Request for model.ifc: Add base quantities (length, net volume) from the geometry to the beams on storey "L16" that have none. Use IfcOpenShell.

First a look at what the model holds.

```python
import ifcopenshell
import ifcopenshell.util.element
import ifcopenshell.util.unit

model = ifcopenshell.open("model.ifc")
print(model.schema)
for unit_type in ("LENGTHUNIT", "AREAUNIT", "VOLUMEUNIT"):
    print(unit_type, ifcopenshell.util.unit.calculate_unit_scale(model, unit_type))
storey = next(s for s in model.by_type("IfcBuildingStorey") if s.Name == "L16")
beams = [e for e in ifcopenshell.util.element.get_decomposition(storey) if e.is_a("IfcBeam")]
for e in sorted(beams, key=lambda e: e.id()):
    print(e.id(), e.is_a(), e.Name, list(ifcopenshell.util.element.get_psets(e, qtos_only=True)), sep=" | ")
```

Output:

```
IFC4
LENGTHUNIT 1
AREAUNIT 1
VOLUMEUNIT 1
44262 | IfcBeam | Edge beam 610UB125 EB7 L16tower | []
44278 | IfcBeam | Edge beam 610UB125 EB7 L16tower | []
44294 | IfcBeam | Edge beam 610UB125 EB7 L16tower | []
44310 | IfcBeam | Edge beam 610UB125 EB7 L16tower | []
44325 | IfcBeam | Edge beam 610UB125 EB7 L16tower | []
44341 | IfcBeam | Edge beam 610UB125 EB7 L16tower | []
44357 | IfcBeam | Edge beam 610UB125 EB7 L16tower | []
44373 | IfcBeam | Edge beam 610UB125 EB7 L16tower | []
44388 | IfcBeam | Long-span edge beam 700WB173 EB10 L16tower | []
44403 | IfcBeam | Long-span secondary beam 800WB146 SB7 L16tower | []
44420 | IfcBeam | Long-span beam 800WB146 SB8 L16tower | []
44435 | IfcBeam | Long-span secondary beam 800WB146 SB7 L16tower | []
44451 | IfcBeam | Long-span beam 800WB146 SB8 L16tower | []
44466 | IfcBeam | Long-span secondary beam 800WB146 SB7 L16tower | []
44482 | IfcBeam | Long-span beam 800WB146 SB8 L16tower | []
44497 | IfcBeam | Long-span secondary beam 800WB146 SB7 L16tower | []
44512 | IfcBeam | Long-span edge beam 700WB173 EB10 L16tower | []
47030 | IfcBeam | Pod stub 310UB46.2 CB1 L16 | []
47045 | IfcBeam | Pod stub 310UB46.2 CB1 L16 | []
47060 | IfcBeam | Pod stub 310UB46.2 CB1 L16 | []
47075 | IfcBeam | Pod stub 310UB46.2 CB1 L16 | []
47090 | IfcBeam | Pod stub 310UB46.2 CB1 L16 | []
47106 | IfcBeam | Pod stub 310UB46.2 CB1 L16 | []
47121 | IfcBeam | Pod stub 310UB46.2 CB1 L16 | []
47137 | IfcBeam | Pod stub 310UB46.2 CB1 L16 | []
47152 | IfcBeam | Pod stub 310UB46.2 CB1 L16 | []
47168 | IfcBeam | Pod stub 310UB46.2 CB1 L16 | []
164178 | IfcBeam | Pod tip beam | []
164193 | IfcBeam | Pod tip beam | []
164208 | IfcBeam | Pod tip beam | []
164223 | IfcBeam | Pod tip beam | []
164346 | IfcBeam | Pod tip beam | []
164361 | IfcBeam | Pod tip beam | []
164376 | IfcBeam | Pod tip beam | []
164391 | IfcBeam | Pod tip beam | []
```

```python
import ifcopenshell
import ifcopenshell.api.pset
import ifcopenshell.geom
import ifcopenshell.util.element
import ifcopenshell.util.shape
import ifcopenshell.util.unit

model = ifcopenshell.open("model.ifc")
unit_scale = ifcopenshell.util.unit.calculate_unit_scale(model)
volume_scale = ifcopenshell.util.unit.calculate_unit_scale(model, "VOLUMEUNIT")
settings = ifcopenshell.geom.settings()

storey = next(s for s in model.by_type("IfcBuildingStorey") if s.Name == "L16")
beams = [e for e in ifcopenshell.util.element.get_decomposition(storey) if e.is_a("IfcBeam")]

for e in sorted(beams, key=lambda e: e.id()):
    if ifcopenshell.util.element.get_psets(e, qtos_only=True, should_inherit=False):
        continue
    # Geometry comes back in metres, in the element's own axes.
    shape = ifcopenshell.geom.create_shape(settings, e)
    values = {
        "Length": ifcopenshell.util.shape.get_max_xyz(shape.geometry) / unit_scale,
        "NetVolume": ifcopenshell.util.shape.get_volume(shape.geometry) / volume_scale,
    }
    qto = ifcopenshell.api.pset.add_qto(model, product=e, name="Qto_BeamBaseQuantities")
    ifcopenshell.api.pset.edit_qto(model, qto=qto, properties=values)
    print(e.id(), {k: round(v, 3) for k, v in values.items()})

model.write("model_edited.ifc")
```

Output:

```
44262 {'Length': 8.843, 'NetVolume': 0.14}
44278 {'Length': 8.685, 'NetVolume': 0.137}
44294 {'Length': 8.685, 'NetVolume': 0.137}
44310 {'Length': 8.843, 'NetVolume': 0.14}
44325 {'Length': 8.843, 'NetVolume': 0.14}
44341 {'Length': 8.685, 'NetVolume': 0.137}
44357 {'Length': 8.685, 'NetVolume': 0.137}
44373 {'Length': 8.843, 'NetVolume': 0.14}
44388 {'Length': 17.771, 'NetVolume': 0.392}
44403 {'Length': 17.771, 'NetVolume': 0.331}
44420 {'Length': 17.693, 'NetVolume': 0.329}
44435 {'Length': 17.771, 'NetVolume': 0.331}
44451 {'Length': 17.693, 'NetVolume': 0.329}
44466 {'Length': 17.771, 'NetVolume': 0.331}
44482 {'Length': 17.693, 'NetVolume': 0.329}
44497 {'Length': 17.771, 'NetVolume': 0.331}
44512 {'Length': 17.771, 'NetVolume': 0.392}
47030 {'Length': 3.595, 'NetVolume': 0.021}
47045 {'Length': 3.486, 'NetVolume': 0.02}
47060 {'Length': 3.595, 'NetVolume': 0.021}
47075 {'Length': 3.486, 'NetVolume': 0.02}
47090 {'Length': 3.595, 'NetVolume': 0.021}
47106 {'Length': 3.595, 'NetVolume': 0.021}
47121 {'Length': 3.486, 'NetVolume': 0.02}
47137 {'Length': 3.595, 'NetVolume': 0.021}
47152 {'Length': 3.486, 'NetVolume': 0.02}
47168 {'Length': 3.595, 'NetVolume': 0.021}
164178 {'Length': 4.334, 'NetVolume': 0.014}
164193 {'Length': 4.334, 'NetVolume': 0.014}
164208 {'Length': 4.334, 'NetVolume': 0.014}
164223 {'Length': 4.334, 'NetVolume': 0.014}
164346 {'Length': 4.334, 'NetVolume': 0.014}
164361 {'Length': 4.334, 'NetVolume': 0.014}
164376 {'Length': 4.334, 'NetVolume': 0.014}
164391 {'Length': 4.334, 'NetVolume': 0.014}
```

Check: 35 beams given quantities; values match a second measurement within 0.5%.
